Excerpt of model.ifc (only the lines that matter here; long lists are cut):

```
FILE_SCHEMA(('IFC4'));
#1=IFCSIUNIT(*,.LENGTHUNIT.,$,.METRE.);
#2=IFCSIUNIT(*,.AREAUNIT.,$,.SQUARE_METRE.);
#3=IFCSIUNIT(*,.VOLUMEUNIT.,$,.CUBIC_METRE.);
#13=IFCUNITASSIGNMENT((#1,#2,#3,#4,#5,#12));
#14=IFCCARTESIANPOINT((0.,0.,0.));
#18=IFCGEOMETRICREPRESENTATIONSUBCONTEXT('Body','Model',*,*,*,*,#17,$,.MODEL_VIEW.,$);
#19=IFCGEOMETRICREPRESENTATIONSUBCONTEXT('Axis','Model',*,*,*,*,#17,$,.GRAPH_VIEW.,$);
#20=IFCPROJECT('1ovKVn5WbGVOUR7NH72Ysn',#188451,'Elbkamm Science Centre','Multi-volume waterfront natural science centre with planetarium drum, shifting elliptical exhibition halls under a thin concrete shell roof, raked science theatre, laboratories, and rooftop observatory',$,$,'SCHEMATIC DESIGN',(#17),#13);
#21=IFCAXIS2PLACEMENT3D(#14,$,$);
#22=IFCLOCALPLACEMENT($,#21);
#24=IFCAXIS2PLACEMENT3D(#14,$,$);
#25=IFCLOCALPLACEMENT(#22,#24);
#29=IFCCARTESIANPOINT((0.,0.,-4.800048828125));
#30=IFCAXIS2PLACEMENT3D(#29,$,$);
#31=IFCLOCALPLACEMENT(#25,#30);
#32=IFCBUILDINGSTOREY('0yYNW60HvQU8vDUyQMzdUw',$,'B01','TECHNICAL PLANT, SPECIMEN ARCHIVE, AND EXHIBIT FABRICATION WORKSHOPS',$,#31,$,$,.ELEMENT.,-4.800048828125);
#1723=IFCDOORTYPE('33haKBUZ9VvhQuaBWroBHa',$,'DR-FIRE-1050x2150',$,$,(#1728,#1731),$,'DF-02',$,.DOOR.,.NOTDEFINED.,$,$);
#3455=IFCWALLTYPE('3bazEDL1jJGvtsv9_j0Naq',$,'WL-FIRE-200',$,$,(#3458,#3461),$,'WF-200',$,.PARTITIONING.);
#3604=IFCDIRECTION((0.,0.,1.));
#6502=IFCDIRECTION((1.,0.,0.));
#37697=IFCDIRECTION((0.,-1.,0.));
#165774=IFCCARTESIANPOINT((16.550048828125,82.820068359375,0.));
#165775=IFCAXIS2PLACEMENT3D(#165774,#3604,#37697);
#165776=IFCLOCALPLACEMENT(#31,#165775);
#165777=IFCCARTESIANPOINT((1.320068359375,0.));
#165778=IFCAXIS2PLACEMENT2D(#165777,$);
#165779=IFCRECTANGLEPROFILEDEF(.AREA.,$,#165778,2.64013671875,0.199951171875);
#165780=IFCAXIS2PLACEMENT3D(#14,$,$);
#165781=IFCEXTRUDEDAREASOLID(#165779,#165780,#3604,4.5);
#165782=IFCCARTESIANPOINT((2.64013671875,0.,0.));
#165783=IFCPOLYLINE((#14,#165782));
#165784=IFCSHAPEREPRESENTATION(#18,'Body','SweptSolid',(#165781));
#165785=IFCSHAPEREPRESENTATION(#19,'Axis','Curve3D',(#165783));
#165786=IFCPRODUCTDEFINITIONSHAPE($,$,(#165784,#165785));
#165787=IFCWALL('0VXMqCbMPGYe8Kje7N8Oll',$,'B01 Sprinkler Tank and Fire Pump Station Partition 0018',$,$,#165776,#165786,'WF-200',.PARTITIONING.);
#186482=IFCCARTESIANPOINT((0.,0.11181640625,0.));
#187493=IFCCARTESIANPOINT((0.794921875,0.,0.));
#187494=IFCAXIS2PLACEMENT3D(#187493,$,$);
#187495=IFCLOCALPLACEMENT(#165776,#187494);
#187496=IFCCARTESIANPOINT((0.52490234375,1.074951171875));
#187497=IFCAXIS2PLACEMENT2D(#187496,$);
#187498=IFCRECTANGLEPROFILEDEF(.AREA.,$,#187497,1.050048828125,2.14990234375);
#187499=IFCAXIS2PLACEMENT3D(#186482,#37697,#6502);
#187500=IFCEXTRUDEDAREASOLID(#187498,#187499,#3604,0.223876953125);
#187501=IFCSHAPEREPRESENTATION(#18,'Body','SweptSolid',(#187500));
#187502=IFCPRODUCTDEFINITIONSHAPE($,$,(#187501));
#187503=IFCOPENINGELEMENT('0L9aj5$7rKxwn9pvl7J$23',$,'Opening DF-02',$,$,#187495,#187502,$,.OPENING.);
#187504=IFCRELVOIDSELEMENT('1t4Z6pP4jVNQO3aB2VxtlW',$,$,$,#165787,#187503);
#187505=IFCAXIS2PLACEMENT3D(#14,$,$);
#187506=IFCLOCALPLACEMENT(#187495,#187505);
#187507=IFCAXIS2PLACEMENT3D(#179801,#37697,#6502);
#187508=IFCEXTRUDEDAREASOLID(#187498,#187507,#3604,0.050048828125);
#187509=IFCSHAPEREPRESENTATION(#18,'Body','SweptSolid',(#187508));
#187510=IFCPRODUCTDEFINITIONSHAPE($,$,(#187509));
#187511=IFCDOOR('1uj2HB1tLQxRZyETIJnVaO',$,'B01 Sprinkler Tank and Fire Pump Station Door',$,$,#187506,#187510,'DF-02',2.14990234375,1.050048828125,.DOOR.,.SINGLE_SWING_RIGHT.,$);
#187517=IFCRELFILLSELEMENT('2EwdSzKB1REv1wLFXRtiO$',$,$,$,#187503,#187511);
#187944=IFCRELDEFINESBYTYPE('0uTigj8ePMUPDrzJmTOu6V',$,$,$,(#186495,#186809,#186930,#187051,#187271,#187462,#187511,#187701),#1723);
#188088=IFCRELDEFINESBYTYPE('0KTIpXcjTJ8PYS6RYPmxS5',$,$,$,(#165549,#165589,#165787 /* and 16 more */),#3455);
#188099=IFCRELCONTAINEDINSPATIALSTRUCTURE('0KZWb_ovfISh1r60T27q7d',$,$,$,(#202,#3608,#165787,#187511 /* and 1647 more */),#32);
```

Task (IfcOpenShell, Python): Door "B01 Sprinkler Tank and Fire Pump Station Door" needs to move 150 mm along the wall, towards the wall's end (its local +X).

```python
import ifcopenshell
import ifcopenshell.api.geometry
import ifcopenshell.util.placement

model = ifcopenshell.open("model.ifc")

door = model.by_id(187511)
opening = door.FillsVoids[0].RelatingOpeningElement
wall = opening.VoidsElements[0].RelatingBuildingElement

wall_matrix = ifcopenshell.util.placement.get_local_placement(wall.ObjectPlacement)
shift = wall_matrix[:3, 0] * 0.15
before = ifcopenshell.util.placement.get_local_placement(door.ObjectPlacement)[:3, 3].copy()

# The door is placed relative to its opening, so it follows when the opening moves.
matrix = ifcopenshell.util.placement.get_local_placement(opening.ObjectPlacement)
matrix[:3, 3] += shift
ifcopenshell.api.geometry.edit_object_placement(
    model, product=opening, matrix=matrix, is_si=False, should_transform_children=True
)

after = ifcopenshell.util.placement.get_local_placement(door.ObjectPlacement)[:3, 3]
print("door moved by", (after - before).round(3) + 0.0)

model.write("model_edited.ifc")
```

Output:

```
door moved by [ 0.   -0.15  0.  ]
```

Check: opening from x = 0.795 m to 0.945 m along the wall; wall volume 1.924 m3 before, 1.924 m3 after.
